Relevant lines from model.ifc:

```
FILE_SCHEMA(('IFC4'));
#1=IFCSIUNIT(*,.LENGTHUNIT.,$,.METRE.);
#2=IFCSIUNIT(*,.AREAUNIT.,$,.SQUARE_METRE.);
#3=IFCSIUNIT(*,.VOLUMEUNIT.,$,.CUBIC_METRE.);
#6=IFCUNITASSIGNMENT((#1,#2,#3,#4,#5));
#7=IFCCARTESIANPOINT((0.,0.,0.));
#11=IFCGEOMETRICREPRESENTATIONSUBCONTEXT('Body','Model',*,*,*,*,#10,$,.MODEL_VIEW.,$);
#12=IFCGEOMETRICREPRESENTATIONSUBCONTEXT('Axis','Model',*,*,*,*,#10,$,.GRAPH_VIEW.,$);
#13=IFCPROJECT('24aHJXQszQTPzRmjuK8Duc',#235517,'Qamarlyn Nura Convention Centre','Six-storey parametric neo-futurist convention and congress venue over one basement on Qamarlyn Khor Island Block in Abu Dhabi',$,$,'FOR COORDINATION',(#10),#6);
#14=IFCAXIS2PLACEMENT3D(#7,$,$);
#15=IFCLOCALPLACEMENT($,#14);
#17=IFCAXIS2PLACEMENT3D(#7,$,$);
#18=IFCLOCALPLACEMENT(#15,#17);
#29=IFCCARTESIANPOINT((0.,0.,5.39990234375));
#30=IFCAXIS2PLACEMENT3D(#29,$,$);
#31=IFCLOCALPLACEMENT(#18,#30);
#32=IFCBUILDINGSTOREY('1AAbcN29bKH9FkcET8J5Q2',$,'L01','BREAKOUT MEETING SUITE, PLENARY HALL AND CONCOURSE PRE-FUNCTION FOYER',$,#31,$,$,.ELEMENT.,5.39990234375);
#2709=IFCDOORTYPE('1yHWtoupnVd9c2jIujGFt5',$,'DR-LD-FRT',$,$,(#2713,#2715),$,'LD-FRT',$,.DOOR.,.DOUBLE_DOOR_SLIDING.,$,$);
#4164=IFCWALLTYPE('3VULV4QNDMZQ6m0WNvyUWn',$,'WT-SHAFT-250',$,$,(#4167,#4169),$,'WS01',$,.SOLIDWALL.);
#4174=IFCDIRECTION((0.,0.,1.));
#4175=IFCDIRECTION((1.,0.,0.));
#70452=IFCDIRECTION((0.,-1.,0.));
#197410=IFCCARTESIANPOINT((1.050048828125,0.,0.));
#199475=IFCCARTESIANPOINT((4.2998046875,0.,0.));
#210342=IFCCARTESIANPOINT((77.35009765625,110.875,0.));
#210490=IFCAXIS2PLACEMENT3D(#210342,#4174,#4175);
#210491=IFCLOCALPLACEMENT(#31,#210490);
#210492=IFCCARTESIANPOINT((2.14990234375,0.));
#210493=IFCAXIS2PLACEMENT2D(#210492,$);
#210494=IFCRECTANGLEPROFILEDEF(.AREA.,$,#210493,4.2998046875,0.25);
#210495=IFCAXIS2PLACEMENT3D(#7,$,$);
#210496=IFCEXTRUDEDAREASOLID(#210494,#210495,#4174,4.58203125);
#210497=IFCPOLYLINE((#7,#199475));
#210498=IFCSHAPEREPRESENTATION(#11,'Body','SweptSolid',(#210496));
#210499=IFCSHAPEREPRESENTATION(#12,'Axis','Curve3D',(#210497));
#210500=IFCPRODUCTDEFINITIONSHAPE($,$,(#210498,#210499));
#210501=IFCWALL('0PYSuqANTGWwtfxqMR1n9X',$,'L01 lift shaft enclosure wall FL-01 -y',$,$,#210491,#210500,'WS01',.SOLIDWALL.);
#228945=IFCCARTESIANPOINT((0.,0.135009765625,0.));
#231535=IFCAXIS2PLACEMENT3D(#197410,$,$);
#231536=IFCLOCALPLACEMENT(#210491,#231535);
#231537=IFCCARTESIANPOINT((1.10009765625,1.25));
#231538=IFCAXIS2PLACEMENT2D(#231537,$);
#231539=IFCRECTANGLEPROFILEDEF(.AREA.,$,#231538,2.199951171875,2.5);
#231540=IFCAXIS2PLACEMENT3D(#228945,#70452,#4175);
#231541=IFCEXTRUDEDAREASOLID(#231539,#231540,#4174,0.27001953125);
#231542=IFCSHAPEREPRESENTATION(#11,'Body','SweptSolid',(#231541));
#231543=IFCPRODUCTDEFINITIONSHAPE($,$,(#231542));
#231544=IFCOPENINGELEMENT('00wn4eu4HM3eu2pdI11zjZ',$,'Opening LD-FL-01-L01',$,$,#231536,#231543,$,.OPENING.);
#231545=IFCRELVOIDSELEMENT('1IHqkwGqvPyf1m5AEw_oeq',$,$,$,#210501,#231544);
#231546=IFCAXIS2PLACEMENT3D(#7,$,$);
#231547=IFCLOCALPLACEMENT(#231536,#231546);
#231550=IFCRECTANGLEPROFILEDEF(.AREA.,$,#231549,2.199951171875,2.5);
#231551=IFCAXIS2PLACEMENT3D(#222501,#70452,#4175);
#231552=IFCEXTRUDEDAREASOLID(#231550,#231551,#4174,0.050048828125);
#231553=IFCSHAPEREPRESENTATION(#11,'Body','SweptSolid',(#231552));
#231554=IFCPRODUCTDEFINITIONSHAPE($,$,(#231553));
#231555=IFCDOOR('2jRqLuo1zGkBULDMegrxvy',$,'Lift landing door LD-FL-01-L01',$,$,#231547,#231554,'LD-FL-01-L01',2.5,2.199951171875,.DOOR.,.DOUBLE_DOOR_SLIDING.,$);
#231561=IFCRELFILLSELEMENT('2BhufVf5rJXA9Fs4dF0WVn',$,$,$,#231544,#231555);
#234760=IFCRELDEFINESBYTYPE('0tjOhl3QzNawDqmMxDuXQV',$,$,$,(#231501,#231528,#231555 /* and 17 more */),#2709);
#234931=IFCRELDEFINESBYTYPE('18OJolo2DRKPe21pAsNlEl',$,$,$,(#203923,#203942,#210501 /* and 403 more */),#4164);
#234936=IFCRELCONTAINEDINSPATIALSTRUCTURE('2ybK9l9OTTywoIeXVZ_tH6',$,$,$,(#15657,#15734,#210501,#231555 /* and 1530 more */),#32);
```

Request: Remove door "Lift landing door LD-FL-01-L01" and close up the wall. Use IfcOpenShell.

```python
import ifcopenshell
import ifcopenshell.api.feature
import ifcopenshell.api.root
import ifcopenshell.geom
import ifcopenshell.util.shape

model = ifcopenshell.open("model.ifc")
settings = ifcopenshell.geom.settings()


def volume(element):
    """Net volume in cubic metres, openings subtracted."""
    shape = ifcopenshell.geom.create_shape(settings, element)
    return ifcopenshell.util.shape.get_volume(shape.geometry)


door = model.by_id(231555)
opening = door.FillsVoids[0].RelatingOpeningElement
wall = opening.VoidsElements[0].RelatingBuildingElement
before = volume(wall)

ifcopenshell.api.root.remove_product(model, product=door)
ifcopenshell.api.feature.remove_feature(model, feature=opening)

after = volume(wall)

print(f"wall volume {before:.3f} -> {after:.3f} m3")

model.write("model_v2.ifc")
```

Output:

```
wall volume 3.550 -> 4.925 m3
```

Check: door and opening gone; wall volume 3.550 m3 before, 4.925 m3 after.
